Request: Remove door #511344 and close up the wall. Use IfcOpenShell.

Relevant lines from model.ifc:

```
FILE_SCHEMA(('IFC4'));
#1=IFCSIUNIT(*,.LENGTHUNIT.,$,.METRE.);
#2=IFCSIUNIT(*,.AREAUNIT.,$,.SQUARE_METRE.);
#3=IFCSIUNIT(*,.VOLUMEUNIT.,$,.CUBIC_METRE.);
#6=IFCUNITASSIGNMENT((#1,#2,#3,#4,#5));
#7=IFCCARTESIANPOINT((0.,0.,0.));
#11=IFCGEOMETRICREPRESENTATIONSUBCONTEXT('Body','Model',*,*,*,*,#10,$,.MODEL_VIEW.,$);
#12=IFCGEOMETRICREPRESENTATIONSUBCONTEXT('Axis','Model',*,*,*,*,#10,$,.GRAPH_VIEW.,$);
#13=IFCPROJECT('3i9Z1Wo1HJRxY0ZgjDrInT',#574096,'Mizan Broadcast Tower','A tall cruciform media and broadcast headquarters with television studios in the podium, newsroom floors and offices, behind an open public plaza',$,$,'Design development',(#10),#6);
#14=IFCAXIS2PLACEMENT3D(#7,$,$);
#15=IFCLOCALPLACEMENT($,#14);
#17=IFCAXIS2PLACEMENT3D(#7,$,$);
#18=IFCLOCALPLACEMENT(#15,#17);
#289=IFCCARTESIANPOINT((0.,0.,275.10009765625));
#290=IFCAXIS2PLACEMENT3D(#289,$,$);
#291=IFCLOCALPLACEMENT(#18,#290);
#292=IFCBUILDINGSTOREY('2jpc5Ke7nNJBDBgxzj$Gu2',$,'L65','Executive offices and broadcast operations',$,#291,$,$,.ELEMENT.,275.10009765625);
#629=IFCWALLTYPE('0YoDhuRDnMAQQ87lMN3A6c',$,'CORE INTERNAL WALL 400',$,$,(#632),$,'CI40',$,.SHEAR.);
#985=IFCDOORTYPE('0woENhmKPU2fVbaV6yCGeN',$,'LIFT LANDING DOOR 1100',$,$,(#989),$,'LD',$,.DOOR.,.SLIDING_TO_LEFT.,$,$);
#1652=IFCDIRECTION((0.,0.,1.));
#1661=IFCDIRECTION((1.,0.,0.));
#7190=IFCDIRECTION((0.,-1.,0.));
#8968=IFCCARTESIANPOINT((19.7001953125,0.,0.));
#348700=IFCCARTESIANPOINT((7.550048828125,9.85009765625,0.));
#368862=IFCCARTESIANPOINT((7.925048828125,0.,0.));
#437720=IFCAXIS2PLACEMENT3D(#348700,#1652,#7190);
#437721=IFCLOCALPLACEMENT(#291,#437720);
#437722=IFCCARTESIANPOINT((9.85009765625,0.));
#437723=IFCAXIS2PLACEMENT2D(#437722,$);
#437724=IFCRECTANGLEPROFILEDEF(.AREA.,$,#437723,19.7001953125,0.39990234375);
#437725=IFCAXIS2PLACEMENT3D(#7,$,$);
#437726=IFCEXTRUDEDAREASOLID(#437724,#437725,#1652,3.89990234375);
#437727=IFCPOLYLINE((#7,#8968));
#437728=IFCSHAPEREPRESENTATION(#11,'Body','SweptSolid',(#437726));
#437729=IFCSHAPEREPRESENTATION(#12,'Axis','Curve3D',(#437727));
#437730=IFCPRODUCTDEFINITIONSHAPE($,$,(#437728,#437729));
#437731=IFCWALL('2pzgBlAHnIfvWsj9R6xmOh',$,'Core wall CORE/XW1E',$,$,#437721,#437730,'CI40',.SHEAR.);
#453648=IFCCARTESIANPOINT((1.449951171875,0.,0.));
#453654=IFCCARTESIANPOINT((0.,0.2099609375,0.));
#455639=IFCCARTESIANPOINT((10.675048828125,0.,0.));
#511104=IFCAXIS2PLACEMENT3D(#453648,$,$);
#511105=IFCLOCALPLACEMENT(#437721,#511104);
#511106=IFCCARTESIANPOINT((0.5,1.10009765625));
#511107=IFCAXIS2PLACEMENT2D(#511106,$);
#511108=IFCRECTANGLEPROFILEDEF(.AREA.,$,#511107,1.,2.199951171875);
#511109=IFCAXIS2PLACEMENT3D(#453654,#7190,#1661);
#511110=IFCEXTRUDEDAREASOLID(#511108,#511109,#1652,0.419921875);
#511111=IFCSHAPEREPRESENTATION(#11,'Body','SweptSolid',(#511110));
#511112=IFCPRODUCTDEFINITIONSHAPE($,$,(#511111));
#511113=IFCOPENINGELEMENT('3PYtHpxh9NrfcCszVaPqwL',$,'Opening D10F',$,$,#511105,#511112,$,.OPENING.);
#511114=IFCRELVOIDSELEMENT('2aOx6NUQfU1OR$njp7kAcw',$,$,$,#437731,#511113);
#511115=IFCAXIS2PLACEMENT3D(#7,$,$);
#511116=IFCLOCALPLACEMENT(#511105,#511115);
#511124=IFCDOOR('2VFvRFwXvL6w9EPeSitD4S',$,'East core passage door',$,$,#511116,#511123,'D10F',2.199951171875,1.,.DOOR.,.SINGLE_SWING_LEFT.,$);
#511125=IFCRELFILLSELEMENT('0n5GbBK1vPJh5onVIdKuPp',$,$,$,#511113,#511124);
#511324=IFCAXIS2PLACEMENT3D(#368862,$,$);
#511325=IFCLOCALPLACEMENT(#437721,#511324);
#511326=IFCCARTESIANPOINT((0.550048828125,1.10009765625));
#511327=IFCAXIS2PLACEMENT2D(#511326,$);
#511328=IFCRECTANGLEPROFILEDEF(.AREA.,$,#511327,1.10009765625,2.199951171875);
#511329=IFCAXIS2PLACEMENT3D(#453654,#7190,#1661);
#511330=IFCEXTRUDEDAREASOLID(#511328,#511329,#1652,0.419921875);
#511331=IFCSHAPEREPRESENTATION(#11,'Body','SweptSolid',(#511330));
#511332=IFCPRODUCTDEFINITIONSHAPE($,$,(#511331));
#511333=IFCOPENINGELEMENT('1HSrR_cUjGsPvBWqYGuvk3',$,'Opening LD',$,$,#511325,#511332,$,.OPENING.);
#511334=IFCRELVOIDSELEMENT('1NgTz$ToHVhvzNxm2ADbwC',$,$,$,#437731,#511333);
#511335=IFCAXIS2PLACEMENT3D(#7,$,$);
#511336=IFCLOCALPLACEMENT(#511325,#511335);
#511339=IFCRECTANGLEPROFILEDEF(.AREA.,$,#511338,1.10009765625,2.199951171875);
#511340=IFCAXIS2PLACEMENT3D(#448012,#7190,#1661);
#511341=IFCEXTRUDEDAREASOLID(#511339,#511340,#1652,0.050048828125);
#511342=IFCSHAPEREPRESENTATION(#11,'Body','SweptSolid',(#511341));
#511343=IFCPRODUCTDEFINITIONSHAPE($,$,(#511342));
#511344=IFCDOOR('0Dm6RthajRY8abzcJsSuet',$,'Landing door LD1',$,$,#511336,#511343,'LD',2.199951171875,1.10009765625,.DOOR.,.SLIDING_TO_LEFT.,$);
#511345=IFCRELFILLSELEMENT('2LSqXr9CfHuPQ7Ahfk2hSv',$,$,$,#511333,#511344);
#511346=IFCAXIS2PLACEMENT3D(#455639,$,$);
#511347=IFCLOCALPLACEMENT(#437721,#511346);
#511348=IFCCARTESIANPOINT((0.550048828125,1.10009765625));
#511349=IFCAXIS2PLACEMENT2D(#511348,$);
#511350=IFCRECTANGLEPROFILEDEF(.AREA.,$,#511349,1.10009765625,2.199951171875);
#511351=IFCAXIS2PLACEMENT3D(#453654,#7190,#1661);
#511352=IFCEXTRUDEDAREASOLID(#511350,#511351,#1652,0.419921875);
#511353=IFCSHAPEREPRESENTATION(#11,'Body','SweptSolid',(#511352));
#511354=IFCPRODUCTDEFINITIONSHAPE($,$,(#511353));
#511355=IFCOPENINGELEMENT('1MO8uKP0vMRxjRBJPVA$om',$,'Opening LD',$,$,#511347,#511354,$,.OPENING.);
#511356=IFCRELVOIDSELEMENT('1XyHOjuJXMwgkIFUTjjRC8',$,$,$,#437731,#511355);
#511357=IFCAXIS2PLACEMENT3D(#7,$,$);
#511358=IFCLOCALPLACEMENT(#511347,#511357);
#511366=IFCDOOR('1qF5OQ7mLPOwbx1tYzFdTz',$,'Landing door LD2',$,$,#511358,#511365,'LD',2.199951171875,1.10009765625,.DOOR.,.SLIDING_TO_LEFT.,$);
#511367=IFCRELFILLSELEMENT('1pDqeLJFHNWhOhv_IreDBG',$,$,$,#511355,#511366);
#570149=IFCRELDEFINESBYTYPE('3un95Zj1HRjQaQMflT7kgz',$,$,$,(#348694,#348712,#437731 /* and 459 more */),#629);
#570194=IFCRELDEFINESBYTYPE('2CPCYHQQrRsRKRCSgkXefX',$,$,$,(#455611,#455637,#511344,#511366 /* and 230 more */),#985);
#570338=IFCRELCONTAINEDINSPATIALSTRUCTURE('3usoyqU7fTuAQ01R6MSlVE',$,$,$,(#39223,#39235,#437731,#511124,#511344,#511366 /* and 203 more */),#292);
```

```python
import ifcopenshell
import ifcopenshell.api.feature
import ifcopenshell.api.root
import ifcopenshell.geom
import ifcopenshell.util.shape

model = ifcopenshell.open("model.ifc")
settings = ifcopenshell.geom.settings()


def volume(element):
    """Net volume in cubic metres, openings subtracted."""
    shape = ifcopenshell.geom.create_shape(settings, element)
    return ifcopenshell.util.shape.get_volume(shape.geometry)


door = model.by_guid("0Dm6RthajRY8abzcJsSuet")
opening = door.FillsVoids[0].RelatingOpeningElement
wall = opening.VoidsElements[0].RelatingBuildingElement
before = volume(wall)

ifcopenshell.api.root.remove_product(model, product=door)
ifcopenshell.api.feature.remove_feature(model, feature=opening)

after = volume(wall)

print(f"wall volume {before:.3f} -> {after:.3f} m3")

model.write("model_edited.ifc")
```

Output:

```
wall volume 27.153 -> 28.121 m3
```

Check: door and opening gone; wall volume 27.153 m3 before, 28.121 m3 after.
